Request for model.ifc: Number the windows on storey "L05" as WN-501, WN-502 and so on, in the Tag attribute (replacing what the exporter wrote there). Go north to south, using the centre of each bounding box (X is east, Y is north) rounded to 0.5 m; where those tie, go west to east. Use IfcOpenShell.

First a look at what the model holds.

```python
import ifcopenshell
import ifcopenshell.util.element
import ifcopenshell.util.placement

model = ifcopenshell.open("model.ifc")
print(model.schema)
storey = next(s for s in model.by_type("IfcBuildingStorey") if s.Name == "L05")
windows = [e for e in ifcopenshell.util.element.get_decomposition(storey) if e.is_a("IfcWindow")]
for e in sorted(windows, key=lambda e: e.id()):
    origin = ifcopenshell.util.placement.get_local_placement(e.ObjectPlacement)[:3, 3]
    print(e.id(), e.Tag, e.Name, origin.round(2) + 0.0, sep=" | ")
```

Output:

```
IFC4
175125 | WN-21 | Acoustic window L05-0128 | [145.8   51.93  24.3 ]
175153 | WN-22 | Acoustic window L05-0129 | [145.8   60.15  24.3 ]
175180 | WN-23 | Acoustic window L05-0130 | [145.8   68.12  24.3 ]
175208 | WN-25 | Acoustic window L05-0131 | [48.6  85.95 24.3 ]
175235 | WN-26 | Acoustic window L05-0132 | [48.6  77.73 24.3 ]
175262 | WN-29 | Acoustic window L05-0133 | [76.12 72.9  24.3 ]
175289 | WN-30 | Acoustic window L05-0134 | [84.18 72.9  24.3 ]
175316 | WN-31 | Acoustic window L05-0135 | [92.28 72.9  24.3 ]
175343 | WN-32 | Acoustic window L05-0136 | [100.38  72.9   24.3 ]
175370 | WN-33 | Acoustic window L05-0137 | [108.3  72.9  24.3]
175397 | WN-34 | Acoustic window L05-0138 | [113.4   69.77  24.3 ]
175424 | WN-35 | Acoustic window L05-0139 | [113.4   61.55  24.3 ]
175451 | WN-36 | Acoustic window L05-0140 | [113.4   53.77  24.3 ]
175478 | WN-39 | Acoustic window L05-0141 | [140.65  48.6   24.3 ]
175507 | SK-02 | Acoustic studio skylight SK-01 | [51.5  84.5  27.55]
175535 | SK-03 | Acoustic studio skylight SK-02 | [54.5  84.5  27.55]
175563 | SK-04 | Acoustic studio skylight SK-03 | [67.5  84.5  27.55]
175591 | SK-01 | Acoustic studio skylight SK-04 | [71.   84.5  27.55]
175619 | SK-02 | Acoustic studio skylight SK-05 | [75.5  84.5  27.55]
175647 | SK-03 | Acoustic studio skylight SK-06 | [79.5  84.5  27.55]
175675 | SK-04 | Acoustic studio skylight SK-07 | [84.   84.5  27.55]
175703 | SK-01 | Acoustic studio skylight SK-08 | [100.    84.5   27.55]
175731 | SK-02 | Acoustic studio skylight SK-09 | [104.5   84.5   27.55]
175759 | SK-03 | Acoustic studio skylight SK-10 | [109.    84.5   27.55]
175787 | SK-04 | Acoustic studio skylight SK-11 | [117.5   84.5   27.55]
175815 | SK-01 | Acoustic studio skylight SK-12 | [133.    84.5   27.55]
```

```python
import ifcopenshell
import ifcopenshell.geom
import ifcopenshell.util.element
import ifcopenshell.util.shape

model = ifcopenshell.open("model.ifc")
settings = ifcopenshell.geom.settings()
settings.set("use-world-coords", True)


def centre(element):
    shape = ifcopenshell.geom.create_shape(settings, element)
    return ifcopenshell.util.shape.get_bbox_centroid(shape.geometry)


storey = next(s for s in model.by_type("IfcBuildingStorey") if s.Name == "L05")
windows = [e for e in ifcopenshell.util.element.get_decomposition(storey) if e.is_a("IfcWindow")]

# Insertion points can sit at a corner or the storey origin, so sort by the geometry (in metres).
centres = {e: centre(e) for e in windows}
windows.sort(key=lambda e: (-round(centres[e][1] / 0.5), centres[e][0]))

for i, e in enumerate(windows, start=1):
    number = f"WN-5{i:02d}"
    e.Tag = number
    print(e.id(), number)

model.write("model_rev.ifc")
```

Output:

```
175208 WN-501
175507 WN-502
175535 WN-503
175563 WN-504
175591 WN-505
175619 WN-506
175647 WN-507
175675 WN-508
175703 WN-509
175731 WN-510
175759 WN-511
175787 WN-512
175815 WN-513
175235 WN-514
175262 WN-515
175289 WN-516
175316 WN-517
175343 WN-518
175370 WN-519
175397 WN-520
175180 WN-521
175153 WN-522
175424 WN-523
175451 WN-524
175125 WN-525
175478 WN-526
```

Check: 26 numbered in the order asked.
